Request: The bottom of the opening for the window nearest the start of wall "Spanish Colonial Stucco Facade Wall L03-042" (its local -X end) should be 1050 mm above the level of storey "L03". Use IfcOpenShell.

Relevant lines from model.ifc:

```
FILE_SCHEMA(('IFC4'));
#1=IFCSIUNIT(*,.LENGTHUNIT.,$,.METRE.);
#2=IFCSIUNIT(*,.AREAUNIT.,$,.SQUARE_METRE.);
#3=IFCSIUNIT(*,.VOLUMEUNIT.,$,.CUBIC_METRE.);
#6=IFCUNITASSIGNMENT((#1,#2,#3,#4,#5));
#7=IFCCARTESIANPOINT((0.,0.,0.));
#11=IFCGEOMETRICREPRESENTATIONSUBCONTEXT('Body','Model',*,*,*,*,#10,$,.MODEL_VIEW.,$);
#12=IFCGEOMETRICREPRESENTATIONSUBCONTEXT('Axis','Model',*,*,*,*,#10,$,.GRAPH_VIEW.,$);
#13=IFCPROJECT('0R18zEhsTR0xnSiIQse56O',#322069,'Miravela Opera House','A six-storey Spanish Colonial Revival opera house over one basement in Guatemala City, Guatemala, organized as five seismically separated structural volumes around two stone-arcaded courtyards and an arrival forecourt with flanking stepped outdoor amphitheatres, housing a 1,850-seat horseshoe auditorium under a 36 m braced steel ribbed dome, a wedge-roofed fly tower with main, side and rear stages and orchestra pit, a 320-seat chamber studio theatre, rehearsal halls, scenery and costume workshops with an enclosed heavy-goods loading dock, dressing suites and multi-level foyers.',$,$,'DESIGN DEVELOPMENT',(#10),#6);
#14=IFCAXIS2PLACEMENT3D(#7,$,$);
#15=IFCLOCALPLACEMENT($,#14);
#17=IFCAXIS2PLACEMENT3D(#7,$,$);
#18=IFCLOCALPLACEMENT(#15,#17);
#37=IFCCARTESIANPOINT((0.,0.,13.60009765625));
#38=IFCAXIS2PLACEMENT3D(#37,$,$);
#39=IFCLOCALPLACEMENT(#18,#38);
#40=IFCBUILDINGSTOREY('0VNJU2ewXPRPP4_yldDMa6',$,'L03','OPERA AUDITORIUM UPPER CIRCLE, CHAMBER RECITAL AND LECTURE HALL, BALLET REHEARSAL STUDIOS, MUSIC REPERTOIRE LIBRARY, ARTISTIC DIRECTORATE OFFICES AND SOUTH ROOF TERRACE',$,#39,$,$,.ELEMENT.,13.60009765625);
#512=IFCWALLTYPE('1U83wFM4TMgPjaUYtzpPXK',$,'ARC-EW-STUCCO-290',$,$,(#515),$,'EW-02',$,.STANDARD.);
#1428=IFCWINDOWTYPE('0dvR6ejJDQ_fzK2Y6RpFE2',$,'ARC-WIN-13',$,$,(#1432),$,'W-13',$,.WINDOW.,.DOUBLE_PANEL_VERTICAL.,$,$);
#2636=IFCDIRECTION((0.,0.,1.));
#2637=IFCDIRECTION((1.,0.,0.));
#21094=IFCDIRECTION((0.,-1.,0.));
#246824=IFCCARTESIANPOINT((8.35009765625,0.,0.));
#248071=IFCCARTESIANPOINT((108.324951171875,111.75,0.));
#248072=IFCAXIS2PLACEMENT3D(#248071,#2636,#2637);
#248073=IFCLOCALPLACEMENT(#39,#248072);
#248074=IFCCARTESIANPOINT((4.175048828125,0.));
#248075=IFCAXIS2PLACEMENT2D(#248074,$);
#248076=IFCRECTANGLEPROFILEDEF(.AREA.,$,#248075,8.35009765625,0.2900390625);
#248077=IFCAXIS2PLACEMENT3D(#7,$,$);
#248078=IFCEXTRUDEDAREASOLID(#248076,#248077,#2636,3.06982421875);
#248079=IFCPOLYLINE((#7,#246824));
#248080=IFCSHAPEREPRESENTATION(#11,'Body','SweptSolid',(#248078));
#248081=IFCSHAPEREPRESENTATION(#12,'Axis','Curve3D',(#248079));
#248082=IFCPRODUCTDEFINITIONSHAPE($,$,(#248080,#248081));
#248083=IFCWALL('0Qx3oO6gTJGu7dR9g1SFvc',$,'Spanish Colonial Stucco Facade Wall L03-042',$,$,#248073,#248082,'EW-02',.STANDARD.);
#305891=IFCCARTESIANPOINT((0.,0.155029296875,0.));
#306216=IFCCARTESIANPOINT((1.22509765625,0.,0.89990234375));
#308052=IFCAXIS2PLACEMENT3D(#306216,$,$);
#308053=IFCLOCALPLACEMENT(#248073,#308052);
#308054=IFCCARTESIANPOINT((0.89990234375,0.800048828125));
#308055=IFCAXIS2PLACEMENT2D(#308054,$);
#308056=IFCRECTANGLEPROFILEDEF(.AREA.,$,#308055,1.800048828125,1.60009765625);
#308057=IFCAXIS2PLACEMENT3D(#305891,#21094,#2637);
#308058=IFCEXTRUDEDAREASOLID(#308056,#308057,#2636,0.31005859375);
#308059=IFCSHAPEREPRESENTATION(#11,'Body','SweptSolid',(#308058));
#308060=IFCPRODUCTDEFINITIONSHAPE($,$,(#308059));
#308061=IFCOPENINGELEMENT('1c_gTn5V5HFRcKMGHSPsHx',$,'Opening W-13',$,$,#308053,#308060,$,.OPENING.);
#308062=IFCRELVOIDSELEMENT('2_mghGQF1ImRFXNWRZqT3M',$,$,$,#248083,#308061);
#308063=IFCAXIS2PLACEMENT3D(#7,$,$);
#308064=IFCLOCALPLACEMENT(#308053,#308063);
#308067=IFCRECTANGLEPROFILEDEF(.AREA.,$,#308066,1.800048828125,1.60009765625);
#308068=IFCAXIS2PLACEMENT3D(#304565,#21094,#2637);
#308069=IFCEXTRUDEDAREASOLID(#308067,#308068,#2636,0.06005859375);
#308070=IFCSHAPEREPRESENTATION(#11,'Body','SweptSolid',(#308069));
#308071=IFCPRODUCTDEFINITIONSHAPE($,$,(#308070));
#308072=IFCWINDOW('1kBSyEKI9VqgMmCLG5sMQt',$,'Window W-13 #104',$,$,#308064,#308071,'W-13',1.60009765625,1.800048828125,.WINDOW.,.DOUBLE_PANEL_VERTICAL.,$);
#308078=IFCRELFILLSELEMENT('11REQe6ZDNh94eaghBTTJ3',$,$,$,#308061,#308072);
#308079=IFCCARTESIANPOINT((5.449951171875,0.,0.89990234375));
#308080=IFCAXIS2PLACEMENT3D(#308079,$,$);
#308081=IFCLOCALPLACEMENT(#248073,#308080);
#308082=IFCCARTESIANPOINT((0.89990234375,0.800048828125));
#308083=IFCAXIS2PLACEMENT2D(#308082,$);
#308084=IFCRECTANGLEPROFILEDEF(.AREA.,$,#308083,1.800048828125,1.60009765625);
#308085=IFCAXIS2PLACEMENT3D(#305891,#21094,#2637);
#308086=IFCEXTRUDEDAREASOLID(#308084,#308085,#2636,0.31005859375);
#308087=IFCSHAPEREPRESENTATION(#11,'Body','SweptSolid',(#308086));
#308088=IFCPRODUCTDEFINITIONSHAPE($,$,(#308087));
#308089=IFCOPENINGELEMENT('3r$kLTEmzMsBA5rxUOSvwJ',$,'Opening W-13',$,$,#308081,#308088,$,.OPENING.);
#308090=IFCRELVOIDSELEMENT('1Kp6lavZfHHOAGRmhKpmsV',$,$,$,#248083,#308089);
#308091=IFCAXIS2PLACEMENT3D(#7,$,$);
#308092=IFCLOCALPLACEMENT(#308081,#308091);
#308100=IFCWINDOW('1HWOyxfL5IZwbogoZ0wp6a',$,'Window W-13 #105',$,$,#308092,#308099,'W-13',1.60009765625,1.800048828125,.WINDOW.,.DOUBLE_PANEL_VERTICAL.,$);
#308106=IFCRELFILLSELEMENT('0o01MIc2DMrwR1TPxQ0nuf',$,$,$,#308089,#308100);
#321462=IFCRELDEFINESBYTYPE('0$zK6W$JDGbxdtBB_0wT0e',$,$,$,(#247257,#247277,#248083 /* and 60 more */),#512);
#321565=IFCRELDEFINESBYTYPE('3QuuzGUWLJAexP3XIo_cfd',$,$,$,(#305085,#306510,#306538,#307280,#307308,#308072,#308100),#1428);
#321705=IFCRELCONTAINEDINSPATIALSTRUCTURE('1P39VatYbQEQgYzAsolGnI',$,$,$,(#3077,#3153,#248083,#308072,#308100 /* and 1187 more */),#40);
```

```python
import numpy as np
import ifcopenshell
import ifcopenshell.api.geometry
import ifcopenshell.geom
import ifcopenshell.util.element
import ifcopenshell.util.placement
import ifcopenshell.util.shape
import ifcopenshell.util.unit

model = ifcopenshell.open("model.ifc")
unit_scale = ifcopenshell.util.unit.calculate_unit_scale(model)

window = model.by_guid("1kBSyEKI9VqgMmCLG5sMQt")
opening = window.FillsVoids[0].RelatingOpeningElement
storey = ifcopenshell.util.element.get_container(window, ifc_class="IfcBuildingStorey")
level = ifcopenshell.util.placement.get_local_placement(storey.ObjectPlacement)[2, 3]

# The opening's origin need not be at the sill, so measure its lowest point.
shape = ifcopenshell.geom.create_shape(ifcopenshell.geom.settings(), opening)
bottom = ifcopenshell.util.shape.get_shape_bottom_elevation(shape, shape.geometry) / unit_scale
dz = level + 1.05 - bottom

shift = np.array([0.0, 0.0, dz])
# The window is placed relative to its opening, so it follows when the opening moves.
matrix = ifcopenshell.util.placement.get_local_placement(opening.ObjectPlacement)
matrix[:3, 3] += shift
ifcopenshell.api.geometry.edit_object_placement(
    model, product=opening, matrix=matrix, is_si=False, should_transform_children=True
)

print(f"moved by {dz * unit_scale:+.3f} m")

model.write("model_v2.ifc")
```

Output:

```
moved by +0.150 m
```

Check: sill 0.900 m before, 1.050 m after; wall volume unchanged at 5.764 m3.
